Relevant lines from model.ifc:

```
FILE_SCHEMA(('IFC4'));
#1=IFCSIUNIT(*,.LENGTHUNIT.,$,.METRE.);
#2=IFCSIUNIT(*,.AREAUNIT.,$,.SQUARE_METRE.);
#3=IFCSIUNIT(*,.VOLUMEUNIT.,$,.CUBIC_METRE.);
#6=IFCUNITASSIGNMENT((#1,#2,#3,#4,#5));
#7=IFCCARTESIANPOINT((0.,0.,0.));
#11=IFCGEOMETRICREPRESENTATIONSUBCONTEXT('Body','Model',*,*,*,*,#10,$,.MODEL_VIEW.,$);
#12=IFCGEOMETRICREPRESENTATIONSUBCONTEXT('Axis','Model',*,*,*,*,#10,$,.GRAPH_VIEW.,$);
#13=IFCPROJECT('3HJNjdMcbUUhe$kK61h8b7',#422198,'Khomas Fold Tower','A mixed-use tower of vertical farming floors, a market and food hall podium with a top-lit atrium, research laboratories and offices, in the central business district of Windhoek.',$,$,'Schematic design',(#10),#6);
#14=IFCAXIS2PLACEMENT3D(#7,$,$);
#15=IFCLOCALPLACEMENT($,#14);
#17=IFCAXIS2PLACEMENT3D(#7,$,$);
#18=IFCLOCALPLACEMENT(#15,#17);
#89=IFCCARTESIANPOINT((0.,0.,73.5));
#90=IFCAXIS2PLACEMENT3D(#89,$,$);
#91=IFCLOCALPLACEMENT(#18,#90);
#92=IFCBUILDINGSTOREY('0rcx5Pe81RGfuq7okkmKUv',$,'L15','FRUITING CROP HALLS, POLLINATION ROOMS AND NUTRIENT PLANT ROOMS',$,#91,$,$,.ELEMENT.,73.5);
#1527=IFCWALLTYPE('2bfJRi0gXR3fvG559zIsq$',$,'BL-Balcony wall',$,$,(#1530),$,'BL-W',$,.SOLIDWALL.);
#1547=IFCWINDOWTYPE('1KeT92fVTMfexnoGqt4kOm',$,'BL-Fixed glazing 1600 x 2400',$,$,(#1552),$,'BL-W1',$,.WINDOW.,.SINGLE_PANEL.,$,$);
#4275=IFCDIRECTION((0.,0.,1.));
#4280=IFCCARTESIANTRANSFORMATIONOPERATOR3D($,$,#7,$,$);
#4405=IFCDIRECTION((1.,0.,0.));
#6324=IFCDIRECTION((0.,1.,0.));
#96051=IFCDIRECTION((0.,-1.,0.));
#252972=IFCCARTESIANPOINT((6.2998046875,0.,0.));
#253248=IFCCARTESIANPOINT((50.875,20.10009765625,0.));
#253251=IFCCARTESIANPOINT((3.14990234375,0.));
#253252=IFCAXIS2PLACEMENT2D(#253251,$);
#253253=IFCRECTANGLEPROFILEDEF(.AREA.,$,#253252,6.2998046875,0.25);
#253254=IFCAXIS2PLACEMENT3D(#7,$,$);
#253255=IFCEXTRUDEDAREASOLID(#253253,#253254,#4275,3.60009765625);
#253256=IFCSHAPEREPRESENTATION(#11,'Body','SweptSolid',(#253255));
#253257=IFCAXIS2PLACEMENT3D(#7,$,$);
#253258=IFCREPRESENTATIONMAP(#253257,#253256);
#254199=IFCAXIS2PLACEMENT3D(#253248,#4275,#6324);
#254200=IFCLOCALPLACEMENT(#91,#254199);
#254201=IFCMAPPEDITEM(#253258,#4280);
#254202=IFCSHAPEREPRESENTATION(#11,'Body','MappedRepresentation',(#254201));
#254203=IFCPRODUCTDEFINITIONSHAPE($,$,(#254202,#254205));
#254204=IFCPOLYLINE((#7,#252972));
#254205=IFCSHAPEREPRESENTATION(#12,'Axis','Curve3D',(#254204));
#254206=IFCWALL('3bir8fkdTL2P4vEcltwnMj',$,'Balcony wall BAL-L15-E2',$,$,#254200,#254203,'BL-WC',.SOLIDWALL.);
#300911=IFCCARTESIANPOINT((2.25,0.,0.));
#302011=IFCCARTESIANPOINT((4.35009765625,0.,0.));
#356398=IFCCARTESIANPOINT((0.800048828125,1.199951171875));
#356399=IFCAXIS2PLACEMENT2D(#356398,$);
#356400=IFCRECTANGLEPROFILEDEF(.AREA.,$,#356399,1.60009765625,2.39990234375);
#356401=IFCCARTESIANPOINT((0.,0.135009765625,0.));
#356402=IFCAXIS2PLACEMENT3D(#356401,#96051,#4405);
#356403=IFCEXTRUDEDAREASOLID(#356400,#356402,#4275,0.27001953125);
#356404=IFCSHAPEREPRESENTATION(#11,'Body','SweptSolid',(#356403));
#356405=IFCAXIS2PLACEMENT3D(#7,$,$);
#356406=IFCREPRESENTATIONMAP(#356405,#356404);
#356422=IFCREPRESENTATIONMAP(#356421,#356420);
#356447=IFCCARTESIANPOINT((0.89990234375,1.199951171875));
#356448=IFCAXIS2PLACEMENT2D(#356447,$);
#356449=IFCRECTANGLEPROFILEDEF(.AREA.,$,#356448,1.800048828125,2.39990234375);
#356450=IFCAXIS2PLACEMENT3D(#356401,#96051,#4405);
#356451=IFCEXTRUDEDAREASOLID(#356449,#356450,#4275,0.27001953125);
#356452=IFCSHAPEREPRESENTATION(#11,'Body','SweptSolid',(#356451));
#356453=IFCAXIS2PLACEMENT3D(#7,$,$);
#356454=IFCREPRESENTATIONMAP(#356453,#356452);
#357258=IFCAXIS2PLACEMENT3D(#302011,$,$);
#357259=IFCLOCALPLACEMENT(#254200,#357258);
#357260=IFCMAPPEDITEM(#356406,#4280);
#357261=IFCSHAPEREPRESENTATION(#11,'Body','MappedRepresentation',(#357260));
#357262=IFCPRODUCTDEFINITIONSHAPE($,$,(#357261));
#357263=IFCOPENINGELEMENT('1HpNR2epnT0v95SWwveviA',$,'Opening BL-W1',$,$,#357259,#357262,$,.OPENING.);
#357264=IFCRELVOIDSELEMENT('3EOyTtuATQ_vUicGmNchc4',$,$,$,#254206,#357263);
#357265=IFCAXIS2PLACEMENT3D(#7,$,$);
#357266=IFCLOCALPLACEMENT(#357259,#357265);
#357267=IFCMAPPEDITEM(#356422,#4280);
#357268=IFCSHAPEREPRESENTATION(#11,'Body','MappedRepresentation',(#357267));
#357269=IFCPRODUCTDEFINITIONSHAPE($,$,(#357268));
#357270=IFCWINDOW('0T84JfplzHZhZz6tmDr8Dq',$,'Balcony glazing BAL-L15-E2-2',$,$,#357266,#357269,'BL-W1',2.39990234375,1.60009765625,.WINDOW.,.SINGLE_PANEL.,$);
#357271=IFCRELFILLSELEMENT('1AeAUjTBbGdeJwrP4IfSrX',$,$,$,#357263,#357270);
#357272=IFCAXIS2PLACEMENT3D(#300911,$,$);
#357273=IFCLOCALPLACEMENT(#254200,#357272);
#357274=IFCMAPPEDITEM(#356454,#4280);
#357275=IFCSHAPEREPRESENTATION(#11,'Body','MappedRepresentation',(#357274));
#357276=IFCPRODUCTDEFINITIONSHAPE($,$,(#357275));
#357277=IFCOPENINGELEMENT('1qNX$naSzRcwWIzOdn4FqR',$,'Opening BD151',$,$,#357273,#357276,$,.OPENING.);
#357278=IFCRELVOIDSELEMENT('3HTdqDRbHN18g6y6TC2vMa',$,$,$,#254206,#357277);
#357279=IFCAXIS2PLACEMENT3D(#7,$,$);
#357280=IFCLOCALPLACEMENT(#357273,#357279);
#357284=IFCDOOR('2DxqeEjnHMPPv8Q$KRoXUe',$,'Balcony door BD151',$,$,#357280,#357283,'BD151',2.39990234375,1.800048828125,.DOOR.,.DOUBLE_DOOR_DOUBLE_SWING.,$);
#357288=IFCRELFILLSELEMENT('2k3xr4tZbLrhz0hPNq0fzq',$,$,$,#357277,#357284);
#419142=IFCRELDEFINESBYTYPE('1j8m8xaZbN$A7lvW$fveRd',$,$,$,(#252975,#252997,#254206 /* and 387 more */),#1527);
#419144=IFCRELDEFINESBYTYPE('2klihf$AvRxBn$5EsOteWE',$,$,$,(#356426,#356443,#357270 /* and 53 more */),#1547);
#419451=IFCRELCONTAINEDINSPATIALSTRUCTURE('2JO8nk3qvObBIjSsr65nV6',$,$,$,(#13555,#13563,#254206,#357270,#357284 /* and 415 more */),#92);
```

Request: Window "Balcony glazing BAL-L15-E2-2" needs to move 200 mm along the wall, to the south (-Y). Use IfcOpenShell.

```python
import ifcopenshell
import ifcopenshell.api.geometry
import ifcopenshell.util.placement
import ifcopenshell.util.unit

model = ifcopenshell.open("model.ifc")
unit_scale = ifcopenshell.util.unit.calculate_unit_scale(model)

window = model.by_guid("0T84JfplzHZhZz6tmDr8Dq")
opening = window.FillsVoids[0].RelatingOpeningElement
wall = opening.VoidsElements[0].RelatingBuildingElement

wall_matrix = ifcopenshell.util.placement.get_local_placement(wall.ObjectPlacement)
shift = wall_matrix[:3, 0] * -0.2 / unit_scale
before = ifcopenshell.util.placement.get_local_placement(window.ObjectPlacement)[:3, 3].copy()

# The window is placed relative to its opening, so it follows when the opening moves.
matrix = ifcopenshell.util.placement.get_local_placement(opening.ObjectPlacement)
matrix[:3, 3] += shift
ifcopenshell.api.geometry.edit_object_placement(
    model, product=opening, matrix=matrix, is_si=False, should_transform_children=True
)

after = ifcopenshell.util.placement.get_local_placement(window.ObjectPlacement)[:3, 3]
print("window moved by", (after - before).round(3) + 0.0)

model.write("model-out.ifc")
```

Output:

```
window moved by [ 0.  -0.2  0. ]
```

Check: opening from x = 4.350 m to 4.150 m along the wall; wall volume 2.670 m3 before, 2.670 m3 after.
